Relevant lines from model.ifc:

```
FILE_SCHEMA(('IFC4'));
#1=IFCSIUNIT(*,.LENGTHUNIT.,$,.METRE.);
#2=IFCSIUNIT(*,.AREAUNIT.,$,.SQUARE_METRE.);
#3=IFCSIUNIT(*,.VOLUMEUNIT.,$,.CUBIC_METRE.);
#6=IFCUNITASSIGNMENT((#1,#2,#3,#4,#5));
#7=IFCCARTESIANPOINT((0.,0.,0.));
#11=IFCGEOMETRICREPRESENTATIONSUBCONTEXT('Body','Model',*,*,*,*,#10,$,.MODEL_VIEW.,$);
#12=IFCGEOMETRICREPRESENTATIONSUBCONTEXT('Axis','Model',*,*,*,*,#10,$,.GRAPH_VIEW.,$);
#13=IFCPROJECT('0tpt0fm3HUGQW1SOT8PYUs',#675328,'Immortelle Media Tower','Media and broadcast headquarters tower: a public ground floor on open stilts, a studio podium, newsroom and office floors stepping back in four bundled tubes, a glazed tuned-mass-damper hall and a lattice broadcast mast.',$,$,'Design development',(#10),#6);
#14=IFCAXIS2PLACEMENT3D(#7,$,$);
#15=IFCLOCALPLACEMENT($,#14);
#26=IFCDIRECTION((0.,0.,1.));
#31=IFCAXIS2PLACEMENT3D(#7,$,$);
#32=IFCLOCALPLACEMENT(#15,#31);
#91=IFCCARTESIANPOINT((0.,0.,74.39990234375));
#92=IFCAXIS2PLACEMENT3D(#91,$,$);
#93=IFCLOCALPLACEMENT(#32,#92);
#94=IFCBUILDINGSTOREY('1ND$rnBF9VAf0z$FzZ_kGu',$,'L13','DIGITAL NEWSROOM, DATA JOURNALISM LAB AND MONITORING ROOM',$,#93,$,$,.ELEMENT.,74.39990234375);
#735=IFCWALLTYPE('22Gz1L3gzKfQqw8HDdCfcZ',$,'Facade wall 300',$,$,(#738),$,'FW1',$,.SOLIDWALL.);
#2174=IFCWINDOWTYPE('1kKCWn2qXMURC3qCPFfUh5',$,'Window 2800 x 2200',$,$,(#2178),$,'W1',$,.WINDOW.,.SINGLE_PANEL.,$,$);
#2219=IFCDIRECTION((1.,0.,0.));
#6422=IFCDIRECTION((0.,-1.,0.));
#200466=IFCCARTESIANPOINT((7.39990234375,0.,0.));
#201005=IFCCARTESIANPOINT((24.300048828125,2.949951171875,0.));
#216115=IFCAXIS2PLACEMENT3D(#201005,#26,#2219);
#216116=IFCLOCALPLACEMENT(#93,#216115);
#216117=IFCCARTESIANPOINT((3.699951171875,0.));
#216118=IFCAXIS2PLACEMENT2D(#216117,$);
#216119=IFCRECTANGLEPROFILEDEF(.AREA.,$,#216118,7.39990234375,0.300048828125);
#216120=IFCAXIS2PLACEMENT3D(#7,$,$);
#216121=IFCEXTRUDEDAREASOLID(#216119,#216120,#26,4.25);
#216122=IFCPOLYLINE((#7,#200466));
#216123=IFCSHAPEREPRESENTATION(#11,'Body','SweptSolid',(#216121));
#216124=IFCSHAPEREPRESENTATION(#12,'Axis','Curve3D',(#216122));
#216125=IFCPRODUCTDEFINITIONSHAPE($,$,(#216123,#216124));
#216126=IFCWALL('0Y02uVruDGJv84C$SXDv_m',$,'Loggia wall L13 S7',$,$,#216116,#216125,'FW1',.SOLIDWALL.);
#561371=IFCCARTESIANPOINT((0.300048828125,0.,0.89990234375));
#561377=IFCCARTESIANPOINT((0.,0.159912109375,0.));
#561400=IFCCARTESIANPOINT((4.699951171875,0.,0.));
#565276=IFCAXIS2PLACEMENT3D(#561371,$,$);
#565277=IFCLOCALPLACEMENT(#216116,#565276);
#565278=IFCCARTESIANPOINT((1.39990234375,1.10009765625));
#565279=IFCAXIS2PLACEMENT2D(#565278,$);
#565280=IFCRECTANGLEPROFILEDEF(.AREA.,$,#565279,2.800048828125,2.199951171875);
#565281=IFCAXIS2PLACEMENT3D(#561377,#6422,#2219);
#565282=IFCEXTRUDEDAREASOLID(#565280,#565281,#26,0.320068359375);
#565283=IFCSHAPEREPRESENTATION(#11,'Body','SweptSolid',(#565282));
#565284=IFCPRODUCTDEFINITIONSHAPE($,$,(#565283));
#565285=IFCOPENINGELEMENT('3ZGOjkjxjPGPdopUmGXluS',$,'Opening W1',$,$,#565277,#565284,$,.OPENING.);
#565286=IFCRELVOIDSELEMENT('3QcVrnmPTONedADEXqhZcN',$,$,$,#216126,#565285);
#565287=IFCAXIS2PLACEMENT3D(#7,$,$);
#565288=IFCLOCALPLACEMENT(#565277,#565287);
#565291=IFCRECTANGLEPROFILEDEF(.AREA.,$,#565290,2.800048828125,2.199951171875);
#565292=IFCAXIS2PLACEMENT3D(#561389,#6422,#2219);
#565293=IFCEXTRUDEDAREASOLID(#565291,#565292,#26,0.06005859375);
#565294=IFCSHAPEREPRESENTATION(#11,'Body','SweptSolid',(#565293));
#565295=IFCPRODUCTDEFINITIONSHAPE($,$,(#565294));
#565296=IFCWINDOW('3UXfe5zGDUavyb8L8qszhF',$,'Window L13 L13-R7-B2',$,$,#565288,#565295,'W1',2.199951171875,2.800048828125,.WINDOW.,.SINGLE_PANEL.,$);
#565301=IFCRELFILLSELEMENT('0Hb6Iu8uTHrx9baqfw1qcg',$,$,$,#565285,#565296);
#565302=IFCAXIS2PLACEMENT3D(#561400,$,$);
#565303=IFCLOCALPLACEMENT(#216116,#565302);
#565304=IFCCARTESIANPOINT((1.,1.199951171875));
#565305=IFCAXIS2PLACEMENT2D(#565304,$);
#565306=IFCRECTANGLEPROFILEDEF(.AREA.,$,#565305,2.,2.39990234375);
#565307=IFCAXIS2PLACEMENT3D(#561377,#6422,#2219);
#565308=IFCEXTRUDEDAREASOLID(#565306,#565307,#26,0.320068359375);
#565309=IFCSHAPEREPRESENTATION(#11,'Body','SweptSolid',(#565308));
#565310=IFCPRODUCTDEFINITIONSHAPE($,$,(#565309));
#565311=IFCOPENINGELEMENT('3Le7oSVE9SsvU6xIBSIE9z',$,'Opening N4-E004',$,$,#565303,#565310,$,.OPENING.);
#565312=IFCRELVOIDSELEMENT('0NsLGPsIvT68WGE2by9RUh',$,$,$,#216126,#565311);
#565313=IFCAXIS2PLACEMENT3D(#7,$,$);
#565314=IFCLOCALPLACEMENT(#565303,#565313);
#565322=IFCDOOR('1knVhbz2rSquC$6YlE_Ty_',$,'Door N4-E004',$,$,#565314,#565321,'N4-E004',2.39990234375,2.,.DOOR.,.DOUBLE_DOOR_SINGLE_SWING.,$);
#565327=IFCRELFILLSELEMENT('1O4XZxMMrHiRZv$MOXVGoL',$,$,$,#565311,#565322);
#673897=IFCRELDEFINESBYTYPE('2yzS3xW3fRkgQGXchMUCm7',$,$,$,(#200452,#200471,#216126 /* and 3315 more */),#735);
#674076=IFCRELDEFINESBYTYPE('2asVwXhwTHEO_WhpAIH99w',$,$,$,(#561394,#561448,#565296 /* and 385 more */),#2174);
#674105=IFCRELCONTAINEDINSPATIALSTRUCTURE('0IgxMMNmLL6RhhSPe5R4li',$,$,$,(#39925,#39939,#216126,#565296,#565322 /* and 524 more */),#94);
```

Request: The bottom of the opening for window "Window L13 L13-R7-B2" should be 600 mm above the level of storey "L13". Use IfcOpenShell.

```python
import numpy as np
import ifcopenshell
import ifcopenshell.api.geometry
import ifcopenshell.geom
import ifcopenshell.util.element
import ifcopenshell.util.placement
import ifcopenshell.util.shape
import ifcopenshell.util.unit

model = ifcopenshell.open("model.ifc")
unit_scale = ifcopenshell.util.unit.calculate_unit_scale(model)

window = model.by_id(565296)
opening = window.FillsVoids[0].RelatingOpeningElement
storey = ifcopenshell.util.element.get_container(window, ifc_class="IfcBuildingStorey")
level = ifcopenshell.util.placement.get_local_placement(storey.ObjectPlacement)[2, 3]

# The opening's origin need not be at the sill, so measure its lowest point.
shape = ifcopenshell.geom.create_shape(ifcopenshell.geom.settings(), opening)
bottom = ifcopenshell.util.shape.get_shape_bottom_elevation(shape, shape.geometry) / unit_scale
dz = level + 0.6 / unit_scale - bottom

shift = np.array([0.0, 0.0, dz])
# The window is placed relative to its opening, so it follows when the opening moves.
matrix = ifcopenshell.util.placement.get_local_placement(opening.ObjectPlacement)
matrix[:3, 3] += shift
ifcopenshell.api.geometry.edit_object_placement(
    model, product=opening, matrix=matrix, is_si=False, should_transform_children=True
)

print(f"moved by {dz * unit_scale:+.3f} m")

model.write("model_updated.ifc")
```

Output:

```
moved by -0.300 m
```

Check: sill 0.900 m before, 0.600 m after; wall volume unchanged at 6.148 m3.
